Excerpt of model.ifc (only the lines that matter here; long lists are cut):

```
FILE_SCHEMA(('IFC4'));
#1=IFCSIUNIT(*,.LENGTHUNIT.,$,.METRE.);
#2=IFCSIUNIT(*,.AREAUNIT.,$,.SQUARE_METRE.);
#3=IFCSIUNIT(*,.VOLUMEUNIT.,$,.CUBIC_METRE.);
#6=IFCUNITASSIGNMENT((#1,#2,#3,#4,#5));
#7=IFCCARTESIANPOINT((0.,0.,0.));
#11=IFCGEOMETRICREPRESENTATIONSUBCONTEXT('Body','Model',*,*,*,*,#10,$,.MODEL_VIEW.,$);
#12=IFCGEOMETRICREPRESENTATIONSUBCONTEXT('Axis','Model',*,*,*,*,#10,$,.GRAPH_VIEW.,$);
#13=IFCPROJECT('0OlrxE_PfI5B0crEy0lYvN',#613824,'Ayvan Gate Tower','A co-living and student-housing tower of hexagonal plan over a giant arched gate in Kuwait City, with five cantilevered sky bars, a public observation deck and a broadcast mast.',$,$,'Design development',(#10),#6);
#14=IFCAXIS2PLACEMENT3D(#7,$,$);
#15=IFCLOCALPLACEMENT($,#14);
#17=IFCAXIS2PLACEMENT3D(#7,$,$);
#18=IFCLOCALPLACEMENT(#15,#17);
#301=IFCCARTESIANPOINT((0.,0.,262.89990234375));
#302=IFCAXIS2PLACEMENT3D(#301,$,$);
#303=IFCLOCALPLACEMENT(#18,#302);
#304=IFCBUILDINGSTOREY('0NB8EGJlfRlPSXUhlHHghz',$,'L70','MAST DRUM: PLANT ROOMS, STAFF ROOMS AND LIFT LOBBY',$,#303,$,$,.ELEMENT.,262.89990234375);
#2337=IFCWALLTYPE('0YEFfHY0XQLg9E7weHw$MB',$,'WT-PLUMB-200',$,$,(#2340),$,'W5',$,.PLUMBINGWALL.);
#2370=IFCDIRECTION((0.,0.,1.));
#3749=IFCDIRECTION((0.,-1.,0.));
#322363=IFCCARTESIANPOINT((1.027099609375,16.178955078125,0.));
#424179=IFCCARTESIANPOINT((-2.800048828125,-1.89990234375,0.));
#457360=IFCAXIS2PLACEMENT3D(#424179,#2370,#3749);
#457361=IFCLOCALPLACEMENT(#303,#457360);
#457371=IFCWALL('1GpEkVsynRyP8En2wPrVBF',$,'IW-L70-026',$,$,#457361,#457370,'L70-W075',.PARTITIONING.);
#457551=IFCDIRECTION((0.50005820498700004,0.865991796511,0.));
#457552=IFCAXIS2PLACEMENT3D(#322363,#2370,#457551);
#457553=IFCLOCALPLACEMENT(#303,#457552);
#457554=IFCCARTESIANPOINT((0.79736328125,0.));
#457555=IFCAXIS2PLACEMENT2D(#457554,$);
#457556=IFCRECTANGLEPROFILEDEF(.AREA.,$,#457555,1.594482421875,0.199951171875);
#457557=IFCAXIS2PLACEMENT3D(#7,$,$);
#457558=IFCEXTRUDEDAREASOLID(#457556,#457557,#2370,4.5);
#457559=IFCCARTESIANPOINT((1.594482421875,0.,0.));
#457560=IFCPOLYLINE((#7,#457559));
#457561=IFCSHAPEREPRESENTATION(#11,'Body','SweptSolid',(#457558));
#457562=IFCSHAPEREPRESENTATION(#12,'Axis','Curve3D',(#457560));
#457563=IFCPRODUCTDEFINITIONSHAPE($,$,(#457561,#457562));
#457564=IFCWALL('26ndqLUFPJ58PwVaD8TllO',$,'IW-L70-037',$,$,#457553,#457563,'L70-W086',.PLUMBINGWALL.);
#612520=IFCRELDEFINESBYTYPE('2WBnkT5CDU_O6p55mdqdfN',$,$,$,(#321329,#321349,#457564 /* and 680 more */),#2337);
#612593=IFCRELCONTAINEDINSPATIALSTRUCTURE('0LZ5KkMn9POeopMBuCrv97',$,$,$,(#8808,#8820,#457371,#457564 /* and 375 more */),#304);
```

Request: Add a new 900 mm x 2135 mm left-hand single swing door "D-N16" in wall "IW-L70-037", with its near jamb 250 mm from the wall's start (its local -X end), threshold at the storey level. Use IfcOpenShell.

```python
import numpy as np
import ifcopenshell
import ifcopenshell.api.feature
import ifcopenshell.api.geometry
import ifcopenshell.api.root
import ifcopenshell.api.spatial
import ifcopenshell.geom
import ifcopenshell.util.element
import ifcopenshell.util.placement
import ifcopenshell.util.representation
import ifcopenshell.util.shape
import ifcopenshell.util.unit

model = ifcopenshell.open("model.ifc")
unit_scale = ifcopenshell.util.unit.calculate_unit_scale(model)
settings = ifcopenshell.geom.settings()


def volume(element):
    """Net volume in cubic metres, openings subtracted."""
    shape = ifcopenshell.geom.create_shape(settings, element)
    return ifcopenshell.util.shape.get_volume(shape.geometry)


wall = model.by_guid("26ndqLUFPJ58PwVaD8TllO")
storey = ifcopenshell.util.element.get_container(wall, ifc_class="IfcBuildingStorey")
context = ifcopenshell.util.representation.get_context(model, "Model", "Body", "MODEL_VIEW")
before = volume(wall)

width, height, from_end, sill = 0.9, 2.135, 0.25, 0.0  # metres

# The wall runs along its own X axis, and the end named is its -X end.
wall_shape = ifcopenshell.geom.create_shape(settings, wall)
x, y, z = ifcopenshell.util.shape.get_vertices(wall_shape.geometry).T
start = x.min() + from_end
face, thickness = float(y.min()), float(y.max() - y.min())
wall_matrix = ifcopenshell.util.placement.get_local_placement(wall.ObjectPlacement)
level = ifcopenshell.util.placement.get_local_placement(storey.ObjectPlacement)[2, 3]


def in_wall(x, y):
    """Placement at x, y metres in the wall's axes, at sill height."""
    matrix = wall_matrix.copy()
    matrix[:, 3] = wall_matrix @ np.array([x / unit_scale, y / unit_scale, 0.0, 1.0])
    matrix[2, 3] = level + sill / unit_scale
    return matrix


# Opening: a box that overshoots both wall faces by 50 mm.
opening = ifcopenshell.api.root.create_entity(model, ifc_class="IfcOpeningElement", predefined_type="OPENING")
box = ifcopenshell.api.geometry.add_wall_representation(
    model, context=context, length=width, height=height, thickness=thickness + 0.1
)
ifcopenshell.api.geometry.assign_representation(model, product=opening, representation=box)
ifcopenshell.api.geometry.edit_object_placement(model, product=opening, matrix=in_wall(start, face - 0.05), is_si=False)
ifcopenshell.api.feature.add_feature(model, feature=opening, element=wall)

door = ifcopenshell.api.root.create_entity(model, ifc_class="IfcDoor", name="D-N16", predefined_type="DOOR")
door.OverallWidth, door.OverallHeight = width / unit_scale, height / unit_scale
door.OperationType = "SINGLE_SWING_LEFT"
body = ifcopenshell.api.geometry.add_door_representation(
    model,
    context=context,
    overall_width=door.OverallWidth,
    overall_height=door.OverallHeight,
    operation_type="SINGLE_SWING_LEFT",
    lining_properties={"LiningDepth": thickness / unit_scale, "ThresholdDepth": thickness / unit_scale},
)
ifcopenshell.api.geometry.assign_representation(model, product=door, representation=body)
ifcopenshell.api.spatial.assign_container(model, products=[door], relating_structure=storey)
ifcopenshell.api.feature.add_filling(model, opening=opening, element=door)

# The lining spans the wall, so the door starts at the wall face.
ifcopenshell.api.geometry.edit_object_placement(model, product=door, matrix=in_wall(start, face), is_si=False)

after = volume(wall)

print(f"wall volume {before:.3f} -> {after:.3f} m3")

model.write("model-out.ifc")
```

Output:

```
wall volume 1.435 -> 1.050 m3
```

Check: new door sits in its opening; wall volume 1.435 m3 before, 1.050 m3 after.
